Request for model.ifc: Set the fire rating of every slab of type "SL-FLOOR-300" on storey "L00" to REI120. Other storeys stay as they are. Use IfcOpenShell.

First a look at what the model holds.

```python
import ifcopenshell
import ifcopenshell.util.element

model = ifcopenshell.open("model.ifc")
print(model.schema)
storey = next(s for s in model.by_type("IfcBuildingStorey") if s.Name == "L00")
slabs = [e for e in ifcopenshell.util.element.get_decomposition(storey) if e.is_a("IfcSlab")]
seen = {}
for e in slabs:
    element_type = ifcopenshell.util.element.get_type(e)
    key = (element_type.Name if element_type != e and element_type else None, ifcopenshell.util.element.get_pset(e, "Pset_SlabCommon", "FireRating"))
    seen[key] = seen.get(key, 0) + 1
for (name, value), count in sorted(seen.items(), key=str):
    print(count, "x", name, "|", value)
```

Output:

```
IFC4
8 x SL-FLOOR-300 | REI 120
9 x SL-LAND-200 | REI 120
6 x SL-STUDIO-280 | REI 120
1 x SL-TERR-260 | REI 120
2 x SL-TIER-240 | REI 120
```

```python
import ifcopenshell
import ifcopenshell.api.pset
import ifcopenshell.util.element

model = ifcopenshell.open("model.ifc")

storey = next(s for s in model.by_type("IfcBuildingStorey") if s.Name == "L00")
slabs = [e for e in ifcopenshell.util.element.get_decomposition(storey) if e.is_a("IfcSlab")]

count = 0
for e in slabs:
    element_type = ifcopenshell.util.element.get_type(e)
    if element_type in (None, e) or element_type.Name != "SL-FLOOR-300":
        continue
    # add_pset returns the element's existing set when there is one.
    pset = ifcopenshell.api.pset.add_pset(model, product=e, name="Pset_SlabCommon")
    ifcopenshell.api.pset.edit_pset(model, pset=pset, properties={"FireRating": "REI120"})
    count += 1

print(count, "slabs updated")

model.write("model_edited.ifc")
```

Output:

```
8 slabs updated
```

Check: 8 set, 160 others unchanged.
